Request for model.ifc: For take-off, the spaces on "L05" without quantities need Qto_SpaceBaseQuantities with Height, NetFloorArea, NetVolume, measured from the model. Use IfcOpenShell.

First a look at what the model holds.

```python
import ifcopenshell
import ifcopenshell.util.element
import ifcopenshell.util.unit

model = ifcopenshell.open("model.ifc")
print(model.schema)
for unit_type in ("LENGTHUNIT", "AREAUNIT", "VOLUMEUNIT"):
    print(unit_type, ifcopenshell.util.unit.calculate_unit_scale(model, unit_type))
storey = next(s for s in model.by_type("IfcBuildingStorey") if s.Name == "L05")
spaces = [e for e in ifcopenshell.util.element.get_decomposition(storey) if e.is_a("IfcSpace")]
for e in sorted(spaces, key=lambda e: e.id()):
    print(e.id(), e.is_a(), e.Name, list(ifcopenshell.util.element.get_psets(e, qtos_only=True)), sep=" | ")
```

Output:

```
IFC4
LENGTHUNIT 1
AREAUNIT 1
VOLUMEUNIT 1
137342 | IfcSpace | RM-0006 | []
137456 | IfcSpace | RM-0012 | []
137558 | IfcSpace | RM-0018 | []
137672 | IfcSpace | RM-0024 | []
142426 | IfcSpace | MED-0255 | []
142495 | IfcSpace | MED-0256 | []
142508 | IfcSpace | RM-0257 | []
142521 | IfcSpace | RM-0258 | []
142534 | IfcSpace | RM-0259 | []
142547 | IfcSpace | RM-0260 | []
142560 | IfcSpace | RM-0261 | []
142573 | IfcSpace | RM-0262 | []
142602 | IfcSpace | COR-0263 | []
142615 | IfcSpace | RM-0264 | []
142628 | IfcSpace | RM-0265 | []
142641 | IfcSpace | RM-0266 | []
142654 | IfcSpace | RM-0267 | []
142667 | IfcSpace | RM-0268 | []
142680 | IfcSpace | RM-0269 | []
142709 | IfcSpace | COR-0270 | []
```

```python
import ifcopenshell
import ifcopenshell.api.pset
import ifcopenshell.geom
import ifcopenshell.util.element
import ifcopenshell.util.shape
import ifcopenshell.util.unit

model = ifcopenshell.open("model.ifc")
unit_scale = ifcopenshell.util.unit.calculate_unit_scale(model)
area_scale = ifcopenshell.util.unit.calculate_unit_scale(model, "AREAUNIT")
volume_scale = ifcopenshell.util.unit.calculate_unit_scale(model, "VOLUMEUNIT")
settings = ifcopenshell.geom.settings()

storey = next(s for s in model.by_type("IfcBuildingStorey") if s.Name == "L05")
spaces = [e for e in ifcopenshell.util.element.get_decomposition(storey) if e.is_a("IfcSpace")]

for e in sorted(spaces, key=lambda e: e.id()):
    if ifcopenshell.util.element.get_psets(e, qtos_only=True, should_inherit=False):
        continue
    # Geometry comes back in metres, in the element's own axes.
    shape = ifcopenshell.geom.create_shape(settings, e)
    values = {
        "Height": ifcopenshell.util.shape.get_z(shape.geometry) / unit_scale,
        "NetFloorArea": ifcopenshell.util.shape.get_footprint_area(shape.geometry) / area_scale,
        "NetVolume": ifcopenshell.util.shape.get_volume(shape.geometry) / volume_scale,
    }
    qto = ifcopenshell.api.pset.add_qto(model, product=e, name="Qto_SpaceBaseQuantities")
    ifcopenshell.api.pset.edit_qto(model, qto=qto, properties=values)
    print(e.id(), {k: round(v, 3) for k, v in values.items()})

model.write("model_rev.ifc")
```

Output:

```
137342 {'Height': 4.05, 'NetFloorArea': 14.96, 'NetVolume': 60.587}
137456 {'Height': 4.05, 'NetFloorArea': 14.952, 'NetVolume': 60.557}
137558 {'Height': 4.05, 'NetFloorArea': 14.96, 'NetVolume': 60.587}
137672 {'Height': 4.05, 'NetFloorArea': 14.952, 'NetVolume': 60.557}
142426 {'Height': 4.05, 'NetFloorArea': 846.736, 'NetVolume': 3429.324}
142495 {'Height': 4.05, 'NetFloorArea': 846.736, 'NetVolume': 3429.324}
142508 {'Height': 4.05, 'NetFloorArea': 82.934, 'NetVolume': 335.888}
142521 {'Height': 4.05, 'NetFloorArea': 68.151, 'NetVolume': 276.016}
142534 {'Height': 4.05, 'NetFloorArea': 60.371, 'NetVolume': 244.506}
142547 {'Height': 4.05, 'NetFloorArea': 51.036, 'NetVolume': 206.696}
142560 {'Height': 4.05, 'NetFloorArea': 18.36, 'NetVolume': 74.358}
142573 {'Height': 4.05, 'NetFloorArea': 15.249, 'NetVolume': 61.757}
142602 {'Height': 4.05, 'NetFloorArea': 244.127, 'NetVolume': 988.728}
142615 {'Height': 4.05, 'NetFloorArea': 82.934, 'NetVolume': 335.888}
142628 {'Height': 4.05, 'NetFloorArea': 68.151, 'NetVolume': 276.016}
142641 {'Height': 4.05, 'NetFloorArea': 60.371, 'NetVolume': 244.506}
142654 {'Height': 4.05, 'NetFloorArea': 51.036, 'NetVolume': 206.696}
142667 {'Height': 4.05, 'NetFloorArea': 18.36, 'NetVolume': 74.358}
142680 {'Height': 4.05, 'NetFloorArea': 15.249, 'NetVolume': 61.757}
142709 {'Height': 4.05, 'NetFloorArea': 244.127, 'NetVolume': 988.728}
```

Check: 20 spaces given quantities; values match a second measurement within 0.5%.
